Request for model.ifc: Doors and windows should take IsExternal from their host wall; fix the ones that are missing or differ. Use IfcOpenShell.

First a look at what the model holds.

```python
import ifcopenshell
import ifcopenshell.util.element

model = ifcopenshell.open("model.ifc")
print(model.schema)
seen = {}
for e in model.by_type("IfcDoor") + model.by_type("IfcWindow"):
    if not e.FillsVoids:
        continue
    host = e.FillsVoids[0].RelatingOpeningElement.VoidsElements[0].RelatingBuildingElement
    own = ifcopenshell.util.element.get_pset(e, f"Pset_{e.is_a()[3:].removesuffix('StandardCase')}Common", "IsExternal")
    wall = ifcopenshell.util.element.get_pset(host, "Pset_WallCommon", "IsExternal")
    seen[e.is_a(), own, wall] = seen.get((e.is_a(), own, wall), 0) + 1
for (cls, own, wall), count in sorted(seen.items(), key=str):
    print(count, cls, "IsExternal:", own, "| host wall:", wall)
```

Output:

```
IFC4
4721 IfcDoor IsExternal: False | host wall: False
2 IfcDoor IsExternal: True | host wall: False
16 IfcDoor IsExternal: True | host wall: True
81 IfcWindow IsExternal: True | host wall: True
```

```python
import ifcopenshell
import ifcopenshell.api.pset
import ifcopenshell.util.element

model = ifcopenshell.open("model.ifc")

count = 0
for ifc_class, pset_name in (("IfcDoor", "Pset_DoorCommon"), ("IfcWindow", "Pset_WindowCommon")):
    for e in model.by_type(ifc_class):
        if not e.FillsVoids:
            continue
        host = e.FillsVoids[0].RelatingOpeningElement.VoidsElements[0].RelatingBuildingElement
        external = ifcopenshell.util.element.get_pset(host, "Pset_WallCommon", "IsExternal")
        if external is None or ifcopenshell.util.element.get_pset(e, pset_name, "IsExternal") == external:
            continue
        pset = ifcopenshell.api.pset.add_pset(model, product=e, name=pset_name)
        ifcopenshell.api.pset.edit_pset(model, pset=pset, properties={"IsExternal": external})
        count += 1

print(count, "updated")

model.write("model_updated.ifc")
```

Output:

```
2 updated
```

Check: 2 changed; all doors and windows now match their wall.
